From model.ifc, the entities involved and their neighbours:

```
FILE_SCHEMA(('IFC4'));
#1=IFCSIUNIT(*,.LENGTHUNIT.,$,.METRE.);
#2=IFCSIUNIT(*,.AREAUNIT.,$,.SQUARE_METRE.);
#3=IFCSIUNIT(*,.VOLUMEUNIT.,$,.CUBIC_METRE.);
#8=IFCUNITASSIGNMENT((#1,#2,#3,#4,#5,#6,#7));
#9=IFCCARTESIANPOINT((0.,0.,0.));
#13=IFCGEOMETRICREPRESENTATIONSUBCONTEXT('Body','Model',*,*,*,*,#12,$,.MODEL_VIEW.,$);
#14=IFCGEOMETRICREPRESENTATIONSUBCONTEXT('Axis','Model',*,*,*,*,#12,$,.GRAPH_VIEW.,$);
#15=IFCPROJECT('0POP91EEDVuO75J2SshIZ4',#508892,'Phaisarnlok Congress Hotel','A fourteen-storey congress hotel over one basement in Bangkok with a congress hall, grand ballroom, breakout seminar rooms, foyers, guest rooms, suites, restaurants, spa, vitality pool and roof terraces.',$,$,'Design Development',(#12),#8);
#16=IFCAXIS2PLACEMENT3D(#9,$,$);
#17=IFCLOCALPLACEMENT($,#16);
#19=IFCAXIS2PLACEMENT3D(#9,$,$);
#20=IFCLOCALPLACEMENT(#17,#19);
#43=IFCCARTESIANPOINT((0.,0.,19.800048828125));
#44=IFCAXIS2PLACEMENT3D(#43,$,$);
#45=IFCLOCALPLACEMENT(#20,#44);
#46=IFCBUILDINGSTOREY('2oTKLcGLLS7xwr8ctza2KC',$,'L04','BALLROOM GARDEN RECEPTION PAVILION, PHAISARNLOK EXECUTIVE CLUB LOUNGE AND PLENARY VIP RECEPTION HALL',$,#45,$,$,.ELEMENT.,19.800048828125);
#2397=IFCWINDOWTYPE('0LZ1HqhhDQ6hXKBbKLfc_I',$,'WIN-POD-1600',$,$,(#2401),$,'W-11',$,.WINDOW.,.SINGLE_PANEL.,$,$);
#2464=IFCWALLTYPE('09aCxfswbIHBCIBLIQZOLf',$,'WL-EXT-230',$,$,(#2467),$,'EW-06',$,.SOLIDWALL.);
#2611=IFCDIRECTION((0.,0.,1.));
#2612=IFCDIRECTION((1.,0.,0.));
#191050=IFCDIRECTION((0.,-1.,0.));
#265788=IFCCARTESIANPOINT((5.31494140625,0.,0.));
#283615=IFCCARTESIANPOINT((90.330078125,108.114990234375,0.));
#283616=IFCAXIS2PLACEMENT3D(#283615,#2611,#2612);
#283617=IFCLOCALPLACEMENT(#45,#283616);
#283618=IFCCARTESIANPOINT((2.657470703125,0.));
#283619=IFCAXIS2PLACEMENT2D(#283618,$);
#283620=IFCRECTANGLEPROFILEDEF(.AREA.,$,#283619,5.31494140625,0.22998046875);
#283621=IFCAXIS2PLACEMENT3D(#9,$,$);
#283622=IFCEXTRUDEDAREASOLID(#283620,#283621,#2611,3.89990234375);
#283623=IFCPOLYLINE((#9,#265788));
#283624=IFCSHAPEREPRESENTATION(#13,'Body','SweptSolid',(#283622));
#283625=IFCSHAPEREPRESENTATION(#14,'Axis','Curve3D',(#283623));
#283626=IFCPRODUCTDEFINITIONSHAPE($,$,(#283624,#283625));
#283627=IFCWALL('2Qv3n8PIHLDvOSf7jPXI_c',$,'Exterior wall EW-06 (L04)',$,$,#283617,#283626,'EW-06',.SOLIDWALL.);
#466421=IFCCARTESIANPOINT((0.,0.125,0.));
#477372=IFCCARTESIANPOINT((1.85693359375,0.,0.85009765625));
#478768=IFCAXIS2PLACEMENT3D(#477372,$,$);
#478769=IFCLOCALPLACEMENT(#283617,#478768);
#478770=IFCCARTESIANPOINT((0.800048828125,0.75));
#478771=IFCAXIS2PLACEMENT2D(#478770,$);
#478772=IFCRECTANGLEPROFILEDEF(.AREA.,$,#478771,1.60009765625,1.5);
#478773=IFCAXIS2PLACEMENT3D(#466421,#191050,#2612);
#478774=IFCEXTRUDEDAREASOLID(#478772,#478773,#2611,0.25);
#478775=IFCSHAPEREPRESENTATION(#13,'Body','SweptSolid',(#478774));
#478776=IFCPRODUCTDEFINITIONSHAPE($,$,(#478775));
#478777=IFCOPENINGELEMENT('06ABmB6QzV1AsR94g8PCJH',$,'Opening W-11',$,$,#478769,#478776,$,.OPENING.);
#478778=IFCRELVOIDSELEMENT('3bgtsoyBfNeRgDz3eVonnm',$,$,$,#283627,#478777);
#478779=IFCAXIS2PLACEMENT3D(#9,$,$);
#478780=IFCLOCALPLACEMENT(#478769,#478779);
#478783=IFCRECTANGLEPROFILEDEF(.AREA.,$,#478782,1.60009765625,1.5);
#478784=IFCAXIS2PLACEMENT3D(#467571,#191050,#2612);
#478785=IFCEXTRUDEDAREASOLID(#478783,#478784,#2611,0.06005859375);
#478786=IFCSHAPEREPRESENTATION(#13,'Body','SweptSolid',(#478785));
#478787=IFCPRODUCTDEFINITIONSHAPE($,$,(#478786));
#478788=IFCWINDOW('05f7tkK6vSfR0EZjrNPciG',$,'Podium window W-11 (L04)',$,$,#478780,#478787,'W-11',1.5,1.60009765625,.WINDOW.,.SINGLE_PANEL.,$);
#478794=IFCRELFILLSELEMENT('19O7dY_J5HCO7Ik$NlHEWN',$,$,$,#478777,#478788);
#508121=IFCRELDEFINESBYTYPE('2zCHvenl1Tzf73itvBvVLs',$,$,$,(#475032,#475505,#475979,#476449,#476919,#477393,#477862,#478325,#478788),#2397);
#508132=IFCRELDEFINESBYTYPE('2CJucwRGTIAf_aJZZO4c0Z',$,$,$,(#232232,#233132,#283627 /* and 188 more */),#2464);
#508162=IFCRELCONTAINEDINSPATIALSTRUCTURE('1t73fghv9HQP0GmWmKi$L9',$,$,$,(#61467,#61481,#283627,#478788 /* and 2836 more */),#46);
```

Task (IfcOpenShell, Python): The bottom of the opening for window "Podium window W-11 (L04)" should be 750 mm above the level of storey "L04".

```python
import numpy as np
import ifcopenshell
import ifcopenshell.api.geometry
import ifcopenshell.geom
import ifcopenshell.util.element
import ifcopenshell.util.placement
import ifcopenshell.util.shape
import ifcopenshell.util.unit

model = ifcopenshell.open("model.ifc")
unit_scale = ifcopenshell.util.unit.calculate_unit_scale(model)

window = model.by_id(478788)
opening = window.FillsVoids[0].RelatingOpeningElement
storey = ifcopenshell.util.element.get_container(window, ifc_class="IfcBuildingStorey")
level = ifcopenshell.util.placement.get_local_placement(storey.ObjectPlacement)[2, 3]

# The opening's origin need not be at the sill, so measure its lowest point.
shape = ifcopenshell.geom.create_shape(ifcopenshell.geom.settings(), opening)
bottom = ifcopenshell.util.shape.get_shape_bottom_elevation(shape, shape.geometry) / unit_scale
dz = level + 0.75 / unit_scale - bottom

shift = np.array([0.0, 0.0, dz])
# The window is placed relative to its opening, so it follows when the opening moves.
matrix = ifcopenshell.util.placement.get_local_placement(opening.ObjectPlacement)
matrix[:3, 3] += shift
ifcopenshell.api.geometry.edit_object_placement(
    model, product=opening, matrix=matrix, is_si=False, should_transform_children=True
)

print(f"moved by {dz * unit_scale:+.3f} m")

model.write("model-out.ifc")
```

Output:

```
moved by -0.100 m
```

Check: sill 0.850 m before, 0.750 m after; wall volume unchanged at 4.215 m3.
